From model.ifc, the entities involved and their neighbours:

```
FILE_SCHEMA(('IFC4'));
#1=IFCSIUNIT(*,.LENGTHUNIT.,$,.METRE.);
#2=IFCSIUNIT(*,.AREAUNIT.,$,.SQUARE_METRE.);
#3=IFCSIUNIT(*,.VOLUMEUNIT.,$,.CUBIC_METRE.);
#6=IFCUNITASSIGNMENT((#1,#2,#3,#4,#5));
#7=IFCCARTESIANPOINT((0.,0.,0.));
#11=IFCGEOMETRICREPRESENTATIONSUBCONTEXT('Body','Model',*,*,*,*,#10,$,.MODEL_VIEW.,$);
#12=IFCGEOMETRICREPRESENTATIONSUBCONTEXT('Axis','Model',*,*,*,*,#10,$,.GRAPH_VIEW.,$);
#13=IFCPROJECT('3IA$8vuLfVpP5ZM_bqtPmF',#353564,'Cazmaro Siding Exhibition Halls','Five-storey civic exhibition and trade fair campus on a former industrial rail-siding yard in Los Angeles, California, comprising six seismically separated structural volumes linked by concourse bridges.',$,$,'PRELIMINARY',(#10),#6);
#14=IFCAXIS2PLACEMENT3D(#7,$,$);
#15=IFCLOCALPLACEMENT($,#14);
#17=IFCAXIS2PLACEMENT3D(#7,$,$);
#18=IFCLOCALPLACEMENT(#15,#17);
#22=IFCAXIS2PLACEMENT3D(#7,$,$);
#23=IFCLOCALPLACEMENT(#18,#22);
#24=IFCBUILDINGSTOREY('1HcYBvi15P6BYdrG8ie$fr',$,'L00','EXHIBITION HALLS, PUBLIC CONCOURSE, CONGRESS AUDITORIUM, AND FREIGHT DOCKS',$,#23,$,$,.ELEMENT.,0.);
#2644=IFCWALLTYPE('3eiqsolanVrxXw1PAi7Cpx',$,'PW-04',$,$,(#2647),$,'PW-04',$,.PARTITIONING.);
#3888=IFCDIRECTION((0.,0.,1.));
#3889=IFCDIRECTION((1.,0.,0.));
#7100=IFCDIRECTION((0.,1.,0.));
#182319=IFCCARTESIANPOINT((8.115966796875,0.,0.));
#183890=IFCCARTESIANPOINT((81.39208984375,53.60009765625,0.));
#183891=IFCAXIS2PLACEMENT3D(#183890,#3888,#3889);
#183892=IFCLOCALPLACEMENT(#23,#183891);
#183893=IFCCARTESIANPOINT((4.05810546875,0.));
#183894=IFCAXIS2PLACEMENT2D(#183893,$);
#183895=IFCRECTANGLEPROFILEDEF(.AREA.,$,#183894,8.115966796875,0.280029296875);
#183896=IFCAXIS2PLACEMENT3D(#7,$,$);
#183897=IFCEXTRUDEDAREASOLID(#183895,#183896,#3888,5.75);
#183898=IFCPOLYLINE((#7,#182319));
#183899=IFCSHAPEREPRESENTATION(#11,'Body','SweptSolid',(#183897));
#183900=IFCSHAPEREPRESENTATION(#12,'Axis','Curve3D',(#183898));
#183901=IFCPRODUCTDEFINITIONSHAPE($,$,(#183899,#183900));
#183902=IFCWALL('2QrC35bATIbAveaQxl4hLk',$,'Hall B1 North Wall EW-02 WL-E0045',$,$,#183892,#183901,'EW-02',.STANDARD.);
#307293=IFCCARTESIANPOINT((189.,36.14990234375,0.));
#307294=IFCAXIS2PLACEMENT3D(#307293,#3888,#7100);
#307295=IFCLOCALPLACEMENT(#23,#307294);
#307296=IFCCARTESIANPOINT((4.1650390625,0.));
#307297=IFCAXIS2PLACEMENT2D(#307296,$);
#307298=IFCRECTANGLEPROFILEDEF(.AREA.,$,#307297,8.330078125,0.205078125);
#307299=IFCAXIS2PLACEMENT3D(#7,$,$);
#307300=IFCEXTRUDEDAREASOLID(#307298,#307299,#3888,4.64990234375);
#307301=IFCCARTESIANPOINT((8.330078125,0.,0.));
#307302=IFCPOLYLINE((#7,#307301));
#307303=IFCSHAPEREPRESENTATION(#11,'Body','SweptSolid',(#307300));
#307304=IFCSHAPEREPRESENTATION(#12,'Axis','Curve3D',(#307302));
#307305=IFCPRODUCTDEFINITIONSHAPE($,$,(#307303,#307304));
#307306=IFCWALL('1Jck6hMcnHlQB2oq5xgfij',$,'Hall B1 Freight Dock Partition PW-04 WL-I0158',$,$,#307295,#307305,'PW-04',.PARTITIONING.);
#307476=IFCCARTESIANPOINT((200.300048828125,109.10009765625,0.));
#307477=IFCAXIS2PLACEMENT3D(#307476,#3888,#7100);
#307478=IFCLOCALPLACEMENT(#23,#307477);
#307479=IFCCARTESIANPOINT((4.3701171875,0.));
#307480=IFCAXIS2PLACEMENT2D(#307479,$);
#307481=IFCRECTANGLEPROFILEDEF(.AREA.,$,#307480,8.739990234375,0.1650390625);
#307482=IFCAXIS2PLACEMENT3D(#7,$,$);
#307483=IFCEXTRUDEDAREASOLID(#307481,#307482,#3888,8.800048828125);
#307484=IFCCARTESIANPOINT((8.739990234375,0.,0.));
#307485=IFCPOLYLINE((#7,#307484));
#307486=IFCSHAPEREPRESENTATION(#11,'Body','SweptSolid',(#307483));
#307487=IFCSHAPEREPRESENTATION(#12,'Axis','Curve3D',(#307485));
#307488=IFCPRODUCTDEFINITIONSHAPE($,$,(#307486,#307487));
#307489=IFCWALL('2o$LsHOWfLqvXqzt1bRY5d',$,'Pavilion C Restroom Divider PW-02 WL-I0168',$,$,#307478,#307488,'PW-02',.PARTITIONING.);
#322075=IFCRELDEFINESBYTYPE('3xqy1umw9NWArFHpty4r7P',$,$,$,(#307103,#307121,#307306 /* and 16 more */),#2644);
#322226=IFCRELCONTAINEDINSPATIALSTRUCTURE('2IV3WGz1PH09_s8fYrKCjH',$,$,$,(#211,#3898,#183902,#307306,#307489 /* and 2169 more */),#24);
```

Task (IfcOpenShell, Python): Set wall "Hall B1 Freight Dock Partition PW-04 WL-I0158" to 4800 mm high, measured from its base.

```python
import ifcopenshell
import ifcopenshell.geom
import ifcopenshell.util.representation
import ifcopenshell.util.shape

model = ifcopenshell.open("model.ifc")
settings = ifcopenshell.geom.settings()


def volume(element):
    """Net volume in cubic metres, openings subtracted."""
    shape = ifcopenshell.geom.create_shape(settings, element)
    return ifcopenshell.util.shape.get_volume(shape.geometry)


wall = model.by_guid("1Jck6hMcnHlQB2oq5xgfij")
before = volume(wall)

body = ifcopenshell.util.representation.get_representation(wall, "Model", "Body")
solid = body.Items[0]
old_height = solid.Depth
solid.Depth = 4.8
after = volume(wall)

print(f"height {old_height:g} -> {solid.Depth:g}, volume {before:.3f} -> {after:.3f} m3")

model.write("model_rev.ifc")
```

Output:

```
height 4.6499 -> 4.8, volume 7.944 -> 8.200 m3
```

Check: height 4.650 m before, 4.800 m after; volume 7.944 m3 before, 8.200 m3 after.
